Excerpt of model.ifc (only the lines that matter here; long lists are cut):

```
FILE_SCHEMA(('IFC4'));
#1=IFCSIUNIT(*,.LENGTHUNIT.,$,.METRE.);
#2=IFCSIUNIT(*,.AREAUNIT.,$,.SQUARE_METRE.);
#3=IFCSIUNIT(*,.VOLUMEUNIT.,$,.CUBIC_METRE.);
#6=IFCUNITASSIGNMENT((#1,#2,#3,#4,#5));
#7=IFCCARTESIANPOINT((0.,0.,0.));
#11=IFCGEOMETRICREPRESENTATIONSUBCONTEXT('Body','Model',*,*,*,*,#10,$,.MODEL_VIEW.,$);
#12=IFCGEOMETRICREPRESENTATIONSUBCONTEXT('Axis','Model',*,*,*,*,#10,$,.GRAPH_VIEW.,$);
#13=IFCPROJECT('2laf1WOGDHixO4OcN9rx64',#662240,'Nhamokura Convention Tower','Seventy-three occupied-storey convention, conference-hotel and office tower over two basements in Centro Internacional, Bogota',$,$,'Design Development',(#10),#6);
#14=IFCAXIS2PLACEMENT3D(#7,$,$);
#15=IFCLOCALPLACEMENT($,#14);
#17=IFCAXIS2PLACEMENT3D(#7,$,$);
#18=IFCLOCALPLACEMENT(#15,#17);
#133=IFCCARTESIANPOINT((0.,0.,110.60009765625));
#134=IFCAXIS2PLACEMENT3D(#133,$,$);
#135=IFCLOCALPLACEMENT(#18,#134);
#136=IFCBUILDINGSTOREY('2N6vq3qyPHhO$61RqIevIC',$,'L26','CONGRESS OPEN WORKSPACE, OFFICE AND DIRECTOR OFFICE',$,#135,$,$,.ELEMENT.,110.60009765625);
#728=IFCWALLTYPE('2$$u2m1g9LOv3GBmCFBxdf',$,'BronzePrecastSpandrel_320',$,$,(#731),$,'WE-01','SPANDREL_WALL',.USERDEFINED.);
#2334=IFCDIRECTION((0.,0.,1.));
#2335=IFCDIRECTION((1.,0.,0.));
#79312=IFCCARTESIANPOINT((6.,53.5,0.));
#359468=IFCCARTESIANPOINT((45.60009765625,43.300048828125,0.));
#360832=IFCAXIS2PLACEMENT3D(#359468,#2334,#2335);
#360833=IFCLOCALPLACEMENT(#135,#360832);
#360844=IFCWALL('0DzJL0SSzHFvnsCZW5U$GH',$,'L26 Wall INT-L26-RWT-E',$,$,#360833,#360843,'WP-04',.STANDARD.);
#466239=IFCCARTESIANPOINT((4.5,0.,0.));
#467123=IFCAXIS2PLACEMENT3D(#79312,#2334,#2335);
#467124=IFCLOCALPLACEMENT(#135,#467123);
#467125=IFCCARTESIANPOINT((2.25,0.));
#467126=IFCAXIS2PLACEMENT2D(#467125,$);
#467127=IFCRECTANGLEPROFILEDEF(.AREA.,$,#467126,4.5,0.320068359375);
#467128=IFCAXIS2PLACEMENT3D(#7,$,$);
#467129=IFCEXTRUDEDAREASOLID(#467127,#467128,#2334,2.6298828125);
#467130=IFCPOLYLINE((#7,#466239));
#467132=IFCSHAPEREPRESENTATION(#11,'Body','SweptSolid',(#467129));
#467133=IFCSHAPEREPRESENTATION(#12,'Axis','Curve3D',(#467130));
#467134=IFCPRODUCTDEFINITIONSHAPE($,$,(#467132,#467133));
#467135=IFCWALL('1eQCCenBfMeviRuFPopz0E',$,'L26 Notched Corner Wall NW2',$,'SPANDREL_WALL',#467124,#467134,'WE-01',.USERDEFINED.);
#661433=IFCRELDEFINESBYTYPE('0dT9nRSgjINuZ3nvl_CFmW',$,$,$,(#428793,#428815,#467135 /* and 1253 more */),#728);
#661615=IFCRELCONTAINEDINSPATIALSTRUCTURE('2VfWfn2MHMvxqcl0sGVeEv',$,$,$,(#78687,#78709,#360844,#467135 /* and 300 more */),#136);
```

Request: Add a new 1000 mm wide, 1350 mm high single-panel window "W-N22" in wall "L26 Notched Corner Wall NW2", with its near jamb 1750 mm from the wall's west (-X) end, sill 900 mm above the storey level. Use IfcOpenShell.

```python
import numpy as np
import ifcopenshell
import ifcopenshell.api.feature
import ifcopenshell.api.geometry
import ifcopenshell.api.root
import ifcopenshell.api.spatial
import ifcopenshell.geom
import ifcopenshell.util.element
import ifcopenshell.util.placement
import ifcopenshell.util.representation
import ifcopenshell.util.shape
import ifcopenshell.util.unit

model = ifcopenshell.open("model.ifc")
unit_scale = ifcopenshell.util.unit.calculate_unit_scale(model)
settings = ifcopenshell.geom.settings()


def volume(element):
    """Net volume in cubic metres, openings subtracted."""
    shape = ifcopenshell.geom.create_shape(settings, element)
    return ifcopenshell.util.shape.get_volume(shape.geometry)


wall = model.by_id(467135)
storey = ifcopenshell.util.element.get_container(wall, ifc_class="IfcBuildingStorey")
context = ifcopenshell.util.representation.get_context(model, "Model", "Body", "MODEL_VIEW")
before = volume(wall)

width, height, from_end, sill = 1, 1.35, 1.75, 0.9  # metres

# The wall runs along its own X axis, and the end named is its -X end.
wall_shape = ifcopenshell.geom.create_shape(settings, wall)
x, y, z = ifcopenshell.util.shape.get_vertices(wall_shape.geometry).T
start = x.min() + from_end
face, thickness = float(y.min()), float(y.max() - y.min())
wall_matrix = ifcopenshell.util.placement.get_local_placement(wall.ObjectPlacement)
level = ifcopenshell.util.placement.get_local_placement(storey.ObjectPlacement)[2, 3]


def in_wall(x, y):
    """Placement at x, y metres in the wall's axes, at sill height."""
    matrix = wall_matrix.copy()
    matrix[:, 3] = wall_matrix @ np.array([x / unit_scale, y / unit_scale, 0.0, 1.0])
    matrix[2, 3] = level + sill / unit_scale
    return matrix


# Opening: a box that overshoots both wall faces by 50 mm.
opening = ifcopenshell.api.root.create_entity(model, ifc_class="IfcOpeningElement", predefined_type="OPENING")
box = ifcopenshell.api.geometry.add_wall_representation(
    model, context=context, length=width, height=height, thickness=thickness + 0.1
)
ifcopenshell.api.geometry.assign_representation(model, product=opening, representation=box)
ifcopenshell.api.geometry.edit_object_placement(model, product=opening, matrix=in_wall(start, face - 0.05), is_si=False)
ifcopenshell.api.feature.add_feature(model, feature=opening, element=wall)

window = ifcopenshell.api.root.create_entity(model, ifc_class="IfcWindow", name="W-N22", predefined_type="WINDOW")
window.OverallWidth, window.OverallHeight = width / unit_scale, height / unit_scale
window.PartitioningType = "SINGLE_PANEL"
body = ifcopenshell.api.geometry.add_window_representation(
    model,
    context=context,
    overall_width=window.OverallWidth,
    overall_height=window.OverallHeight,
    partition_type="SINGLE_PANEL",
)
ifcopenshell.api.geometry.assign_representation(model, product=window, representation=body)
ifcopenshell.api.spatial.assign_container(model, products=[window], relating_structure=storey)
ifcopenshell.api.feature.add_filling(model, opening=opening, element=window)

# Centre the window in the wall's thickness.
ifcopenshell.api.geometry.edit_object_placement(model, product=window, matrix=in_wall(start, face), is_si=False)
window_shape = ifcopenshell.geom.create_shape(settings, window)
depth = ifcopenshell.util.shape.get_vertices(window_shape.geometry)[:, 1]
offset = face + thickness / 2 - (depth.min() + depth.max()) / 2
ifcopenshell.api.geometry.edit_object_placement(model, product=window, matrix=in_wall(start, offset), is_si=False)

after = volume(wall)

print(f"wall volume {before:.3f} -> {after:.3f} m3")

model.write("model_edited.ifc")
```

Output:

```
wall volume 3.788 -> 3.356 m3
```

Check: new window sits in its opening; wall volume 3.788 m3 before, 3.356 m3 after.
